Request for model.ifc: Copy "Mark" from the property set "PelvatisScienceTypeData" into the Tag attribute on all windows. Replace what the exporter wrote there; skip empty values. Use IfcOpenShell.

First a look at what the model holds.

```python
import ifcopenshell
import ifcopenshell.util.element

model = ifcopenshell.open("model.ifc")
print(model.schema)
windows = model.by_type("IfcWindow")
print(len(windows), "windows")
for e in windows[:8]:
    source = ifcopenshell.util.element.get_pset(e, "PelvatisScienceTypeData", "Mark")
    target = e.Tag
    print(e.id(), repr(source), repr(target), sep=" | ")
```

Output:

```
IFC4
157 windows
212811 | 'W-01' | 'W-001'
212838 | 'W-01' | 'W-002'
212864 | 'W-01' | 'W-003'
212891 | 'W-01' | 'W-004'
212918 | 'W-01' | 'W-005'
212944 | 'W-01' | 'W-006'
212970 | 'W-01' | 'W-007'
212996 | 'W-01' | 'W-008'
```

```python
import ifcopenshell
import ifcopenshell.util.element

model = ifcopenshell.open("model.ifc")

count = 0
for e in model.by_type("IfcWindow"):
    value = ifcopenshell.util.element.get_pset(e, "PelvatisScienceTypeData", "Mark")
    current = e.Tag
    if not value or not value.strip() or current == value:
        continue
    e.Tag = value
    count += 1

print(count, "windows updated")

model.write("model-out.ifc")
```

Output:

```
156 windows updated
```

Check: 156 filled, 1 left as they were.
